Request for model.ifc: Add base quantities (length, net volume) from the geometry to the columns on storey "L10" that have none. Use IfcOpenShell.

First a look at what the model holds.

```python
import ifcopenshell
import ifcopenshell.util.element
import ifcopenshell.util.unit

model = ifcopenshell.open("model.ifc")
print(model.schema)
for unit_type in ("LENGTHUNIT", "AREAUNIT", "VOLUMEUNIT"):
    print(unit_type, ifcopenshell.util.unit.calculate_unit_scale(model, unit_type))
storey = next(s for s in model.by_type("IfcBuildingStorey") if s.Name == "L10")
columns = [e for e in ifcopenshell.util.element.get_decomposition(storey) if e.is_a("IfcColumn")]
for e in sorted(columns, key=lambda e: e.id()):
    print(e.id(), e.is_a(), e.Name, list(ifcopenshell.util.element.get_psets(e, qtos_only=True)), sep=" | ")
```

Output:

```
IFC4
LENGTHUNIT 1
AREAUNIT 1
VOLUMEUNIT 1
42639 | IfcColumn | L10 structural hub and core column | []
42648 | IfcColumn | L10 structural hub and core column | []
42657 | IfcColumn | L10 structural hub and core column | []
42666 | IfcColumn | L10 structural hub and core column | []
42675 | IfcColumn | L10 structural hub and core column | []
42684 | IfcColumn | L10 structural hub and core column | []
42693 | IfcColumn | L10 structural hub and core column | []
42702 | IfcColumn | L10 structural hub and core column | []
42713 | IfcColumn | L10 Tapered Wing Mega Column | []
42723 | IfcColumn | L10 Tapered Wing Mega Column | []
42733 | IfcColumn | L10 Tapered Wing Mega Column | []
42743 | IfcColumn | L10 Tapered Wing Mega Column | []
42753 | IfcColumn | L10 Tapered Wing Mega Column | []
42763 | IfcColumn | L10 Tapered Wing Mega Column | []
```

```python
import ifcopenshell
import ifcopenshell.api.pset
import ifcopenshell.geom
import ifcopenshell.util.element
import ifcopenshell.util.shape
import ifcopenshell.util.unit

model = ifcopenshell.open("model.ifc")
unit_scale = ifcopenshell.util.unit.calculate_unit_scale(model)
volume_scale = ifcopenshell.util.unit.calculate_unit_scale(model, "VOLUMEUNIT")
settings = ifcopenshell.geom.settings()

storey = next(s for s in model.by_type("IfcBuildingStorey") if s.Name == "L10")
columns = [e for e in ifcopenshell.util.element.get_decomposition(storey) if e.is_a("IfcColumn")]

for e in sorted(columns, key=lambda e: e.id()):
    if ifcopenshell.util.element.get_psets(e, qtos_only=True, should_inherit=False):
        continue
    # Geometry comes back in metres, in the element's own axes.
    shape = ifcopenshell.geom.create_shape(settings, e)
    values = {
        "Length": ifcopenshell.util.shape.get_z(shape.geometry) / unit_scale,
        "NetVolume": ifcopenshell.util.shape.get_volume(shape.geometry) / volume_scale,
    }
    qto = ifcopenshell.api.pset.add_qto(model, product=e, name="Qto_ColumnBaseQuantities")
    ifcopenshell.api.pset.edit_qto(model, qto=qto, properties=values)
    print(e.id(), {k: round(v, 3) for k, v in values.items()})

model.write("model_v2.ifc")
```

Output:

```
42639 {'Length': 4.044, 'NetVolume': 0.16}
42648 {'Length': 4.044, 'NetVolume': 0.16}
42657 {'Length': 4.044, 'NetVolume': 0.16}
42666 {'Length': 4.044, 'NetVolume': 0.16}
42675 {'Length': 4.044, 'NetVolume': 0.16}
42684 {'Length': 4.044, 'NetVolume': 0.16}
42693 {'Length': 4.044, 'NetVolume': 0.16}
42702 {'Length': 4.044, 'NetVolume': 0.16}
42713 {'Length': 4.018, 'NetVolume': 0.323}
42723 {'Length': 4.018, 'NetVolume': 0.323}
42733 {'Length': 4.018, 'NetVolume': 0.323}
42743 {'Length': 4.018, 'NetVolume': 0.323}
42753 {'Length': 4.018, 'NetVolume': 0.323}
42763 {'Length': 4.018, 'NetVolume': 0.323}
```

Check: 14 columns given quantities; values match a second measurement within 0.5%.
